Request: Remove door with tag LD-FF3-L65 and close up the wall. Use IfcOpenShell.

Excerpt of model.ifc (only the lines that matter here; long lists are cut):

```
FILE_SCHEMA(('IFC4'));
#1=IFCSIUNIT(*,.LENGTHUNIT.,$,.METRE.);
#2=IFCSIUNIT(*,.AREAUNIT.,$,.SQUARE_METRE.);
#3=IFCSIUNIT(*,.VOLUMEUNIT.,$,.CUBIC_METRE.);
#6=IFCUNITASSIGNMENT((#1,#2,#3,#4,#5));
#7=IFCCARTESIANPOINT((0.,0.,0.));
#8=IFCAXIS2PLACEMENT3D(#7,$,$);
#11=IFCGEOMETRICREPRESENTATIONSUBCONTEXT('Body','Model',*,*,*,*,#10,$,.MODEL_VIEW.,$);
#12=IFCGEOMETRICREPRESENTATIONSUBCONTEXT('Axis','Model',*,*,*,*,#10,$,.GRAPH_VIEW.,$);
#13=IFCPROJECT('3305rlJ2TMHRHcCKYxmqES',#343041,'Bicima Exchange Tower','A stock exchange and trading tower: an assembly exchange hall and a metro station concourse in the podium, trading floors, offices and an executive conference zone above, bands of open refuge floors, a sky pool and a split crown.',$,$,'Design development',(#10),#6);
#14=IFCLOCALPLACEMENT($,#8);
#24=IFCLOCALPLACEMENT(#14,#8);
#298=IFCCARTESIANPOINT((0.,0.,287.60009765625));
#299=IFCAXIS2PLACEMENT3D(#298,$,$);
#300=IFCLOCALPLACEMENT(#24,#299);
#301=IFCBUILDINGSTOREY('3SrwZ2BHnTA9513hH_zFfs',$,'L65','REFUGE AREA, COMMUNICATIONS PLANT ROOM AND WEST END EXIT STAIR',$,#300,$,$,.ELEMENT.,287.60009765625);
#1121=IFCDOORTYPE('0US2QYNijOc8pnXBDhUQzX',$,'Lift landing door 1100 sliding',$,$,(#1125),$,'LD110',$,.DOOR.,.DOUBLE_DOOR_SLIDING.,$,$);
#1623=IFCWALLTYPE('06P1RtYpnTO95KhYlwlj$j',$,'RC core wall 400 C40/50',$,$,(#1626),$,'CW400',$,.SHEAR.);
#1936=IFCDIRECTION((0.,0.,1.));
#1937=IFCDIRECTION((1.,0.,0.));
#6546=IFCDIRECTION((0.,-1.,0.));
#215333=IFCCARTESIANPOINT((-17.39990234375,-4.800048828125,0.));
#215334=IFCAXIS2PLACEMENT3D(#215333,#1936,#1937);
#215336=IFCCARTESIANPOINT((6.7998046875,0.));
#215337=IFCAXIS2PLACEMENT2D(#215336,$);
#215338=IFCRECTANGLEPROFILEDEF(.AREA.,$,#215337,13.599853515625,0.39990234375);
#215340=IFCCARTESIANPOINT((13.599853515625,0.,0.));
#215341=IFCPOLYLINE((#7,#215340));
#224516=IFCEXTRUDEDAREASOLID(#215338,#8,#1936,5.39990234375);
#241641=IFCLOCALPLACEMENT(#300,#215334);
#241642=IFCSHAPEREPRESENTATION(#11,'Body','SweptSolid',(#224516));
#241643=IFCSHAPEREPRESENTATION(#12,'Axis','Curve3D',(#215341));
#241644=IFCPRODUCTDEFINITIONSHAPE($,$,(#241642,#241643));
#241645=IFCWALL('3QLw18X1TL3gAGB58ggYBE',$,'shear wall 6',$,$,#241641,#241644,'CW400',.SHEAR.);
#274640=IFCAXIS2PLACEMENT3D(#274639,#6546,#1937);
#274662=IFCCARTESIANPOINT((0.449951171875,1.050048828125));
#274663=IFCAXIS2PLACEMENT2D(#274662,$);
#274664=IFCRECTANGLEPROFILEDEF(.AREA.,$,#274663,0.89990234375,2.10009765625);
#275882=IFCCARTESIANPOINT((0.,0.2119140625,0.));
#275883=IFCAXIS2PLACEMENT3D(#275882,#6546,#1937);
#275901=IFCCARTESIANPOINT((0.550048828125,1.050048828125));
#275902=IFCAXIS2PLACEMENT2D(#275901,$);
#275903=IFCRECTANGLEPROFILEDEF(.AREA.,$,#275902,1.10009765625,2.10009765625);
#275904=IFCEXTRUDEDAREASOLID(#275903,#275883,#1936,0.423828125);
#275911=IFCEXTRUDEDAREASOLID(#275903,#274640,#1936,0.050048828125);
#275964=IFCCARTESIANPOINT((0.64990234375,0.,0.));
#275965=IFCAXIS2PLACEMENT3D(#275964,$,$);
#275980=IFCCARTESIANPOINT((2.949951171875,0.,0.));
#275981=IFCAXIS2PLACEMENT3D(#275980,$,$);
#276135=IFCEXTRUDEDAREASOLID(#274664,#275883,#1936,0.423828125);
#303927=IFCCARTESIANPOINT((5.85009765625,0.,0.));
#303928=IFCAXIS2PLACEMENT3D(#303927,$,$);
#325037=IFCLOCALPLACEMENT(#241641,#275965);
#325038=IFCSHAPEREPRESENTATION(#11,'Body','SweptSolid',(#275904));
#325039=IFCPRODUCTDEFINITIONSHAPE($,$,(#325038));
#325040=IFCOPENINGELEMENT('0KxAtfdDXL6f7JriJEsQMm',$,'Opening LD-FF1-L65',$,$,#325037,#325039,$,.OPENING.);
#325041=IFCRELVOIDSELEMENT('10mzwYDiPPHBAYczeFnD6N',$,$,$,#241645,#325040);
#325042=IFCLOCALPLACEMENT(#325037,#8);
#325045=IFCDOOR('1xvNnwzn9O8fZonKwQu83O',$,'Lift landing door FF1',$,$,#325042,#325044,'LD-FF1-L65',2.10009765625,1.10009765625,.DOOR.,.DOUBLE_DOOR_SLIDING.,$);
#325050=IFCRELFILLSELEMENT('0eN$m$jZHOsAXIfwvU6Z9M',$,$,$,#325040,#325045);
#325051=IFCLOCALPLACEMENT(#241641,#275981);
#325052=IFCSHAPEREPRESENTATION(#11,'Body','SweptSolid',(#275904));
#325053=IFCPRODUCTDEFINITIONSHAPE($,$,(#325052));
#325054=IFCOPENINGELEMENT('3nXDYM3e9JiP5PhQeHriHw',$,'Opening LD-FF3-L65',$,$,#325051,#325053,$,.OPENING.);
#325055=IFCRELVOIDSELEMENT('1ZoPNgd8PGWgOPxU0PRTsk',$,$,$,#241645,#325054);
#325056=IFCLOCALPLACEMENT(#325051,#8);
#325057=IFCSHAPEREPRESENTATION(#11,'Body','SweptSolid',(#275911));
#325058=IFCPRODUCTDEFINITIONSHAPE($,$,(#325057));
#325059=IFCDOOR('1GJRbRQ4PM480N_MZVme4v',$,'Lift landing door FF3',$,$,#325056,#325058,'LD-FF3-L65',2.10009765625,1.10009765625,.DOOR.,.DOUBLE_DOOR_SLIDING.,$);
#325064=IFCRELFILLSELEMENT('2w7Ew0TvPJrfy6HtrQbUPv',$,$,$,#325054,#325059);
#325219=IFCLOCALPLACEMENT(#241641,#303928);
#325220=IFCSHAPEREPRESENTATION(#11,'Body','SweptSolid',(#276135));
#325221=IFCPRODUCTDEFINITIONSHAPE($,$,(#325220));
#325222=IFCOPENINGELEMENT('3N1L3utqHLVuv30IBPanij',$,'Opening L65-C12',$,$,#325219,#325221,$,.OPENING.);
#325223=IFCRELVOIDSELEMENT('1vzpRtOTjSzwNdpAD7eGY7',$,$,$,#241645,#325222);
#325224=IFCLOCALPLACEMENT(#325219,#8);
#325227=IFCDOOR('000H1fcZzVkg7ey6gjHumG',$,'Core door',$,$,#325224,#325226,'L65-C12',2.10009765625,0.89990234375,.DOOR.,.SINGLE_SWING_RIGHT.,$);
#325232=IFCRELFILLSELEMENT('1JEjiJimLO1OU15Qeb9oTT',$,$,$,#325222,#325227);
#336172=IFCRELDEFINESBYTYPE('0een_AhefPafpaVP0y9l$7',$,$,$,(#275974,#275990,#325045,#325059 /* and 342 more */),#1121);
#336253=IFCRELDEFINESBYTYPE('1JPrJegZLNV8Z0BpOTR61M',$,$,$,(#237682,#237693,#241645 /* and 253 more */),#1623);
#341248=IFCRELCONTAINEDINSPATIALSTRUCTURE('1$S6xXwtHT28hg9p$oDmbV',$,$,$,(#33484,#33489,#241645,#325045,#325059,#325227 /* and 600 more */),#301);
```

```python
import ifcopenshell
import ifcopenshell.api.feature
import ifcopenshell.api.root
import ifcopenshell.geom
import ifcopenshell.util.shape

model = ifcopenshell.open("model.ifc")
settings = ifcopenshell.geom.settings()


def volume(element):
    """Net volume in cubic metres, openings subtracted."""
    shape = ifcopenshell.geom.create_shape(settings, element)
    return ifcopenshell.util.shape.get_volume(shape.geometry)


door = model.by_guid("1GJRbRQ4PM480N_MZVme4v")
opening = door.FillsVoids[0].RelatingOpeningElement
wall = opening.VoidsElements[0].RelatingBuildingElement
before = volume(wall)

ifcopenshell.api.root.remove_product(model, product=door)
ifcopenshell.api.feature.remove_feature(model, feature=opening)

after = volume(wall)

print(f"wall volume {before:.3f} -> {after:.3f} m3")

model.write("model-out.ifc")
```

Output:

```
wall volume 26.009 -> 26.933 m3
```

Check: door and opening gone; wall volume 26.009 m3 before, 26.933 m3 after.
